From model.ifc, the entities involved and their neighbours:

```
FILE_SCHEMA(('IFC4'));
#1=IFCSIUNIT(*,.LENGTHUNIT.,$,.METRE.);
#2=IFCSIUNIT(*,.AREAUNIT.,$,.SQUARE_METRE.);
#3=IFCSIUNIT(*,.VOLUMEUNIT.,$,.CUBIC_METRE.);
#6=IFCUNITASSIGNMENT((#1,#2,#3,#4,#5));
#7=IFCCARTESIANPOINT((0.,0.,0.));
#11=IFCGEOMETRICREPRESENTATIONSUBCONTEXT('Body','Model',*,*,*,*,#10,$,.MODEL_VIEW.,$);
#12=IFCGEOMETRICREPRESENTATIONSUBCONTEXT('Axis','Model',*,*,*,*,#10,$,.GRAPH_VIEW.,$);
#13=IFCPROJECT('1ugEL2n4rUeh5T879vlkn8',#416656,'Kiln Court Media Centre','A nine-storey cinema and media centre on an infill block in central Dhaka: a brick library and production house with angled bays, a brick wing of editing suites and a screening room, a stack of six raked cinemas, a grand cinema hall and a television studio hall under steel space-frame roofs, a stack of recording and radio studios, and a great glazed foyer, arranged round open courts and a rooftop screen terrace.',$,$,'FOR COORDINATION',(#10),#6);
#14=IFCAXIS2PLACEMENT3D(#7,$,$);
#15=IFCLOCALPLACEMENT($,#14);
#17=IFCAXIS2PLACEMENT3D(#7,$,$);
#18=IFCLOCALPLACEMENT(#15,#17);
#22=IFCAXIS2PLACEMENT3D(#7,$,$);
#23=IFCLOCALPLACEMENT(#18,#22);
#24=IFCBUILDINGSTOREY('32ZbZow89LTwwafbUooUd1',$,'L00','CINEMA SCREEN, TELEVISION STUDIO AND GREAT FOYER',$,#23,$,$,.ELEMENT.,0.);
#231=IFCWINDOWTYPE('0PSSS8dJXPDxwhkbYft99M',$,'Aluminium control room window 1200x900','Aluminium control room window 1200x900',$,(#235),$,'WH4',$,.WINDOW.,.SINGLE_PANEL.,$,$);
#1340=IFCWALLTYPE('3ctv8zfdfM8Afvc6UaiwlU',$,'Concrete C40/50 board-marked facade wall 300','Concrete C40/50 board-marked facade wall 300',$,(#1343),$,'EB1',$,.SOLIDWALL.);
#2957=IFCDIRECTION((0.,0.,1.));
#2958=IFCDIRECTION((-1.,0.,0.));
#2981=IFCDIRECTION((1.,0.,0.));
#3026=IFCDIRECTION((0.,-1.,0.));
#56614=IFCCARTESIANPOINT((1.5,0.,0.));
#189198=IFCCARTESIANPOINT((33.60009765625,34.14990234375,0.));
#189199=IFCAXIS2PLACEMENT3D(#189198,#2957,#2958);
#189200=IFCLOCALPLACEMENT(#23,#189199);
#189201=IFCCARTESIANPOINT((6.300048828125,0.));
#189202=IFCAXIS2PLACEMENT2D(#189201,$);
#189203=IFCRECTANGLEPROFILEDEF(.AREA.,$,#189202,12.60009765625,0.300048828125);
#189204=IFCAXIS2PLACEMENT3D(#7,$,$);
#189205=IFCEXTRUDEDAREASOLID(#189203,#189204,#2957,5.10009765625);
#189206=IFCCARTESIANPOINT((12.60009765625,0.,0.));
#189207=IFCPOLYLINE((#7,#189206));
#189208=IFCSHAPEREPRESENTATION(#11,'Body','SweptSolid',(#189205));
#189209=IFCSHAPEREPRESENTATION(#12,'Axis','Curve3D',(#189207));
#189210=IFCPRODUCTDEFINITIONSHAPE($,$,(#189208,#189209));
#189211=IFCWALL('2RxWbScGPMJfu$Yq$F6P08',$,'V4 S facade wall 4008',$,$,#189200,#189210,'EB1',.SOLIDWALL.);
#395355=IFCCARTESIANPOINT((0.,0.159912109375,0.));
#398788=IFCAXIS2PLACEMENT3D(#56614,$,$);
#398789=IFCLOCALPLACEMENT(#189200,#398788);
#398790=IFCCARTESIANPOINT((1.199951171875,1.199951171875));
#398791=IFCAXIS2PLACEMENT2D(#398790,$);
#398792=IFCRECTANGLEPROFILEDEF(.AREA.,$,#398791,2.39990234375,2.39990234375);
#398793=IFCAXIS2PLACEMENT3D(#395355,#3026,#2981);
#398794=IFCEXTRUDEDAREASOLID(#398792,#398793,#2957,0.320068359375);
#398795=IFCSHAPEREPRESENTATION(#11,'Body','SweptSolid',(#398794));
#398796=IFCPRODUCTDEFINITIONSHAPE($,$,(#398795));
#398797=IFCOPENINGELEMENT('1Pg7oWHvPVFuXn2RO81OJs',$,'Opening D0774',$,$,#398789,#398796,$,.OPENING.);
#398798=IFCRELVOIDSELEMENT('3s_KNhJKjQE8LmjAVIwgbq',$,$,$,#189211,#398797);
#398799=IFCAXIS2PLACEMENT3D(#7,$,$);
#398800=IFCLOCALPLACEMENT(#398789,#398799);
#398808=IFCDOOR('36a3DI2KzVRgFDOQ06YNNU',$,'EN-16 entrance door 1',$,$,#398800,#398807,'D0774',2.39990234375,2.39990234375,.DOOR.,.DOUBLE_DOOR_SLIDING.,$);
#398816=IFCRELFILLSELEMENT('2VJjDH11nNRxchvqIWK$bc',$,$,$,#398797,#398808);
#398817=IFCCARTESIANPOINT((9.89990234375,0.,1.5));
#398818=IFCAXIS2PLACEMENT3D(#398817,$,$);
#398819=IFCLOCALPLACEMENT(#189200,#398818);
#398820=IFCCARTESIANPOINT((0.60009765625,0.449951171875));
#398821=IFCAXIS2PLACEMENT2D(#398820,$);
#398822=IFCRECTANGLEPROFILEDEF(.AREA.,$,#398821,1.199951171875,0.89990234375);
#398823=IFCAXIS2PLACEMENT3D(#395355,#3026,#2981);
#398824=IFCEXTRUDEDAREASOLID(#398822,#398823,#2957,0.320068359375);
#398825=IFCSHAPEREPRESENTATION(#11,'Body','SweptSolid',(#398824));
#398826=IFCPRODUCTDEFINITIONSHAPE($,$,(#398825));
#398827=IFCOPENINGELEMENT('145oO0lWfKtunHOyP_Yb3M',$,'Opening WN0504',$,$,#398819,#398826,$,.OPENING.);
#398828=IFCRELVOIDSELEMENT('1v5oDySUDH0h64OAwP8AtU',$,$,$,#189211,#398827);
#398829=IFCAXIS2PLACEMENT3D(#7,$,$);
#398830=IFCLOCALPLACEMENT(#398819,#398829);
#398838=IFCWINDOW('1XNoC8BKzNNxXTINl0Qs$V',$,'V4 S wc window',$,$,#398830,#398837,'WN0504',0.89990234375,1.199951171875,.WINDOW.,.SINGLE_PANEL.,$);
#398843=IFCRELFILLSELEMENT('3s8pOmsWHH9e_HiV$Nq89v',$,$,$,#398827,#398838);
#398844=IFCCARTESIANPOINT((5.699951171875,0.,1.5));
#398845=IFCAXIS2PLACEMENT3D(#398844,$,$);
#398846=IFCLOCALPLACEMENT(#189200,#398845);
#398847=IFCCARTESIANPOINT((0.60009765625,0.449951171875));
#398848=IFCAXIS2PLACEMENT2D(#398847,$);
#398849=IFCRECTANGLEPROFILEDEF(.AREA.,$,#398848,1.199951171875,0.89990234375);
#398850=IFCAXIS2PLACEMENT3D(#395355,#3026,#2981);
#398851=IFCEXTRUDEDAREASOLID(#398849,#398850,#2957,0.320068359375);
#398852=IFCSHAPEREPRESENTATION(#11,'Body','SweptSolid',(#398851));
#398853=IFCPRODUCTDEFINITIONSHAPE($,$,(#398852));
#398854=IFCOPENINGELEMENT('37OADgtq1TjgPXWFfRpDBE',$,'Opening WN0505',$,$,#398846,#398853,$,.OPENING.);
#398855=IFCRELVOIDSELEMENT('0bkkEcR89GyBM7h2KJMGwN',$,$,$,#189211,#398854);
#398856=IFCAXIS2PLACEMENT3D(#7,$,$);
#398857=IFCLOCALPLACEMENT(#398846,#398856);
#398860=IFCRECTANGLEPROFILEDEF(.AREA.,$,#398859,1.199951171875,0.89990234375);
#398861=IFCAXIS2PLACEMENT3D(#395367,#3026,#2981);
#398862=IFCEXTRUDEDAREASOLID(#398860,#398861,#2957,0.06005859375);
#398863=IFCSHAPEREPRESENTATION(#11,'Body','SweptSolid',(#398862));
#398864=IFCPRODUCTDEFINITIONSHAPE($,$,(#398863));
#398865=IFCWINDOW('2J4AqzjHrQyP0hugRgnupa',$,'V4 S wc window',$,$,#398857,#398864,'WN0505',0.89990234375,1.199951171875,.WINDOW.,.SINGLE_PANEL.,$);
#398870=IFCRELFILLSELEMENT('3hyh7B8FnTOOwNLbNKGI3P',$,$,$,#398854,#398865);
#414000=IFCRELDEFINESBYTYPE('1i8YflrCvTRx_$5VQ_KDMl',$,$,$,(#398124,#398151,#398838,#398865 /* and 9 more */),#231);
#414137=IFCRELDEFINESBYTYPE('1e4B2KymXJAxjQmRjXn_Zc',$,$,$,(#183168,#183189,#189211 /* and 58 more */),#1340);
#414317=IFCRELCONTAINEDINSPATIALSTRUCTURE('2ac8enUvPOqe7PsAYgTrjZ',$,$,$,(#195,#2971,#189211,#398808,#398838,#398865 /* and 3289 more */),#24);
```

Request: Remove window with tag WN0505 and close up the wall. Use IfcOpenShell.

```python
import ifcopenshell
import ifcopenshell.api.feature
import ifcopenshell.api.root
import ifcopenshell.geom
import ifcopenshell.util.shape

model = ifcopenshell.open("model.ifc")
settings = ifcopenshell.geom.settings()


def volume(element):
    """Net volume in cubic metres, openings subtracted."""
    shape = ifcopenshell.geom.create_shape(settings, element)
    return ifcopenshell.util.shape.get_volume(shape.geometry)


window = model.by_guid("2J4AqzjHrQyP0hugRgnupa")
opening = window.FillsVoids[0].RelatingOpeningElement
wall = opening.VoidsElements[0].RelatingBuildingElement
before = volume(wall)

ifcopenshell.api.root.remove_product(model, product=window)
ifcopenshell.api.feature.remove_feature(model, feature=opening)

after = volume(wall)

print(f"wall volume {before:.3f} -> {after:.3f} m3")

model.write("model_updated.ifc")
```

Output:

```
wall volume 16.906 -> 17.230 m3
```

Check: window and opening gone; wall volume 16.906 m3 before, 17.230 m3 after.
